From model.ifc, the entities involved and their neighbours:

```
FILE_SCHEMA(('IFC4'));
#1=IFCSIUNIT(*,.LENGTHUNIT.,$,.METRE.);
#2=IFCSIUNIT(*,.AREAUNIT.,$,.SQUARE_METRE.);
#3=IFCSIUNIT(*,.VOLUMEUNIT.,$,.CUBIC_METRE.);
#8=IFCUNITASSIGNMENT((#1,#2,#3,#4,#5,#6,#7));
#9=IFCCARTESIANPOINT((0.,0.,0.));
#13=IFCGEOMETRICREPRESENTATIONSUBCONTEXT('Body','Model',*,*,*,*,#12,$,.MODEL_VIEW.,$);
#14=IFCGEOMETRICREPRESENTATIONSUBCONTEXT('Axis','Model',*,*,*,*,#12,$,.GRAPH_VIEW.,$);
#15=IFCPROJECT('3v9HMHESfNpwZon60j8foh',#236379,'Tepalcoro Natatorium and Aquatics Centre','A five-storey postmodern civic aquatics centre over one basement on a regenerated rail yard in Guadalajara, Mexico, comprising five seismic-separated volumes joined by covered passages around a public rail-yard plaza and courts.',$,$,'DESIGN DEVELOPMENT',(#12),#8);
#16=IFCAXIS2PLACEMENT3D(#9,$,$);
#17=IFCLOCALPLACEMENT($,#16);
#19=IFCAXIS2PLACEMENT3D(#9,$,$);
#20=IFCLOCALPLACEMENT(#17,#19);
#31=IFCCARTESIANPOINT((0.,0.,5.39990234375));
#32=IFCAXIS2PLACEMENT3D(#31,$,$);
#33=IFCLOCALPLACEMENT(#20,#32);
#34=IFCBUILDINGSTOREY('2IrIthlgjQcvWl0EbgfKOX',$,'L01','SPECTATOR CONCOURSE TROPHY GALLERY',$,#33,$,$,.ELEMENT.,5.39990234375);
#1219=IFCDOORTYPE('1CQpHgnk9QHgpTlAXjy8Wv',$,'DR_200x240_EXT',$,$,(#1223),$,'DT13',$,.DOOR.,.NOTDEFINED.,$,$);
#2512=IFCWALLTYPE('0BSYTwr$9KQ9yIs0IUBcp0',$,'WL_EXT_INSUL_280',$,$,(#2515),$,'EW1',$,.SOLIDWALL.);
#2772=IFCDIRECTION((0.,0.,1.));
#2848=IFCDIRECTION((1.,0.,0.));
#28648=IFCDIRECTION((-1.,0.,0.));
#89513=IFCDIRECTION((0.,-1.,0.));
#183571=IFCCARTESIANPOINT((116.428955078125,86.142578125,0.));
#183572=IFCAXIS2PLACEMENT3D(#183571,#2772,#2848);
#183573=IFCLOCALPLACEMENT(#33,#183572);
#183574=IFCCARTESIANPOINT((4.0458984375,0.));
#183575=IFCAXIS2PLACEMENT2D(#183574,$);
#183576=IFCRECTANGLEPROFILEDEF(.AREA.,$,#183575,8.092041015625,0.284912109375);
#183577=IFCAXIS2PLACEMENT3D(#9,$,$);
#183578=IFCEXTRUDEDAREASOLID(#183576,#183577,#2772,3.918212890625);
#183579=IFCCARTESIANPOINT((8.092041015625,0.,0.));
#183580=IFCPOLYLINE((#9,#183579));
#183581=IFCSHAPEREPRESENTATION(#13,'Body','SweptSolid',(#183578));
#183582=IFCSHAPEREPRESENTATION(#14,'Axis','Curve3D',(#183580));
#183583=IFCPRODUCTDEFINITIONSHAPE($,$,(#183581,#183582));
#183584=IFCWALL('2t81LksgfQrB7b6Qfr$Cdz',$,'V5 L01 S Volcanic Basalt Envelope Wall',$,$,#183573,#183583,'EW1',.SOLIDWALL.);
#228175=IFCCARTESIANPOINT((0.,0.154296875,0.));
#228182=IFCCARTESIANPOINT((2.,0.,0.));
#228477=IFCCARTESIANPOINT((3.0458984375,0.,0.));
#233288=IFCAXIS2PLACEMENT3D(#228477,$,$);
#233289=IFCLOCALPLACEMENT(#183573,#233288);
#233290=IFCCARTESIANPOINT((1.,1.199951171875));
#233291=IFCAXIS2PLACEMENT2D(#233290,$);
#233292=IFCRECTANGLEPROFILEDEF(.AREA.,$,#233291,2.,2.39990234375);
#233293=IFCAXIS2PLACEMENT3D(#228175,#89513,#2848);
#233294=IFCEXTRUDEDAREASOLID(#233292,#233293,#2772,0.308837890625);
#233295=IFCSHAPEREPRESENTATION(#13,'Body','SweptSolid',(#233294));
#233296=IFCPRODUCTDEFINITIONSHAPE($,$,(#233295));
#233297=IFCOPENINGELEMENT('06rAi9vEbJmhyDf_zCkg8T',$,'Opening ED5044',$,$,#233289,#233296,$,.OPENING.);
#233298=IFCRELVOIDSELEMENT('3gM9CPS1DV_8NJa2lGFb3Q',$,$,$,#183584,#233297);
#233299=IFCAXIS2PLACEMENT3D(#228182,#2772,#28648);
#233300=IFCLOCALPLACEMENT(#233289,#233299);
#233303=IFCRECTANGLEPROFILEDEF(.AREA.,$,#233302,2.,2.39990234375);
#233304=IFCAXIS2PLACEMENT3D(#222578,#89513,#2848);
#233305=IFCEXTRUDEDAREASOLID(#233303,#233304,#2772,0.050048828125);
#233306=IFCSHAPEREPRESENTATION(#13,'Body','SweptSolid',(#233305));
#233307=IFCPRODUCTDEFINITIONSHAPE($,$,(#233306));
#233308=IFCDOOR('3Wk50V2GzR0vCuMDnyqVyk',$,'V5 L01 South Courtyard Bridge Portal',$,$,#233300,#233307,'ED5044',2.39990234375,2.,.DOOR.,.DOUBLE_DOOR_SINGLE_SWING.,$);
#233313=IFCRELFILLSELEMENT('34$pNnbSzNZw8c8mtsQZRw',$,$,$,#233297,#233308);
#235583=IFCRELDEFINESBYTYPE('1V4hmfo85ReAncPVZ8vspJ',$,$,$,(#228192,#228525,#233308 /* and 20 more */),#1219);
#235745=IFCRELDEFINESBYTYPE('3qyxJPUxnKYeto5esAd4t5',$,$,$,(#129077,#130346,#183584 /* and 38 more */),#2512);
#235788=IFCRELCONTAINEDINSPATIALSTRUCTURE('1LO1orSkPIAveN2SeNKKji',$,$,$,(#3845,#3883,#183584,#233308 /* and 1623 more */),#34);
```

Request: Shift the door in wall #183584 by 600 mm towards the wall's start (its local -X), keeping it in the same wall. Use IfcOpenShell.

```python
import ifcopenshell
import ifcopenshell.api.geometry
import ifcopenshell.util.placement

model = ifcopenshell.open("model.ifc")

door = model.by_id(233308)
opening = door.FillsVoids[0].RelatingOpeningElement
wall = opening.VoidsElements[0].RelatingBuildingElement

wall_matrix = ifcopenshell.util.placement.get_local_placement(wall.ObjectPlacement)
shift = wall_matrix[:3, 0] * -0.6
before = ifcopenshell.util.placement.get_local_placement(door.ObjectPlacement)[:3, 3].copy()

# The door is placed relative to its opening, so it follows when the opening moves.
matrix = ifcopenshell.util.placement.get_local_placement(opening.ObjectPlacement)
matrix[:3, 3] += shift
ifcopenshell.api.geometry.edit_object_placement(
    model, product=opening, matrix=matrix, is_si=False, should_transform_children=True
)

after = ifcopenshell.util.placement.get_local_placement(door.ObjectPlacement)[:3, 3]
print("door moved by", (after - before).round(3) + 0.0)

model.write("model_v2.ifc")
```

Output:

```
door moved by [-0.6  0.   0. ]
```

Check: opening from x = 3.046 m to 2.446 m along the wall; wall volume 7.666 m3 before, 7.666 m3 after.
